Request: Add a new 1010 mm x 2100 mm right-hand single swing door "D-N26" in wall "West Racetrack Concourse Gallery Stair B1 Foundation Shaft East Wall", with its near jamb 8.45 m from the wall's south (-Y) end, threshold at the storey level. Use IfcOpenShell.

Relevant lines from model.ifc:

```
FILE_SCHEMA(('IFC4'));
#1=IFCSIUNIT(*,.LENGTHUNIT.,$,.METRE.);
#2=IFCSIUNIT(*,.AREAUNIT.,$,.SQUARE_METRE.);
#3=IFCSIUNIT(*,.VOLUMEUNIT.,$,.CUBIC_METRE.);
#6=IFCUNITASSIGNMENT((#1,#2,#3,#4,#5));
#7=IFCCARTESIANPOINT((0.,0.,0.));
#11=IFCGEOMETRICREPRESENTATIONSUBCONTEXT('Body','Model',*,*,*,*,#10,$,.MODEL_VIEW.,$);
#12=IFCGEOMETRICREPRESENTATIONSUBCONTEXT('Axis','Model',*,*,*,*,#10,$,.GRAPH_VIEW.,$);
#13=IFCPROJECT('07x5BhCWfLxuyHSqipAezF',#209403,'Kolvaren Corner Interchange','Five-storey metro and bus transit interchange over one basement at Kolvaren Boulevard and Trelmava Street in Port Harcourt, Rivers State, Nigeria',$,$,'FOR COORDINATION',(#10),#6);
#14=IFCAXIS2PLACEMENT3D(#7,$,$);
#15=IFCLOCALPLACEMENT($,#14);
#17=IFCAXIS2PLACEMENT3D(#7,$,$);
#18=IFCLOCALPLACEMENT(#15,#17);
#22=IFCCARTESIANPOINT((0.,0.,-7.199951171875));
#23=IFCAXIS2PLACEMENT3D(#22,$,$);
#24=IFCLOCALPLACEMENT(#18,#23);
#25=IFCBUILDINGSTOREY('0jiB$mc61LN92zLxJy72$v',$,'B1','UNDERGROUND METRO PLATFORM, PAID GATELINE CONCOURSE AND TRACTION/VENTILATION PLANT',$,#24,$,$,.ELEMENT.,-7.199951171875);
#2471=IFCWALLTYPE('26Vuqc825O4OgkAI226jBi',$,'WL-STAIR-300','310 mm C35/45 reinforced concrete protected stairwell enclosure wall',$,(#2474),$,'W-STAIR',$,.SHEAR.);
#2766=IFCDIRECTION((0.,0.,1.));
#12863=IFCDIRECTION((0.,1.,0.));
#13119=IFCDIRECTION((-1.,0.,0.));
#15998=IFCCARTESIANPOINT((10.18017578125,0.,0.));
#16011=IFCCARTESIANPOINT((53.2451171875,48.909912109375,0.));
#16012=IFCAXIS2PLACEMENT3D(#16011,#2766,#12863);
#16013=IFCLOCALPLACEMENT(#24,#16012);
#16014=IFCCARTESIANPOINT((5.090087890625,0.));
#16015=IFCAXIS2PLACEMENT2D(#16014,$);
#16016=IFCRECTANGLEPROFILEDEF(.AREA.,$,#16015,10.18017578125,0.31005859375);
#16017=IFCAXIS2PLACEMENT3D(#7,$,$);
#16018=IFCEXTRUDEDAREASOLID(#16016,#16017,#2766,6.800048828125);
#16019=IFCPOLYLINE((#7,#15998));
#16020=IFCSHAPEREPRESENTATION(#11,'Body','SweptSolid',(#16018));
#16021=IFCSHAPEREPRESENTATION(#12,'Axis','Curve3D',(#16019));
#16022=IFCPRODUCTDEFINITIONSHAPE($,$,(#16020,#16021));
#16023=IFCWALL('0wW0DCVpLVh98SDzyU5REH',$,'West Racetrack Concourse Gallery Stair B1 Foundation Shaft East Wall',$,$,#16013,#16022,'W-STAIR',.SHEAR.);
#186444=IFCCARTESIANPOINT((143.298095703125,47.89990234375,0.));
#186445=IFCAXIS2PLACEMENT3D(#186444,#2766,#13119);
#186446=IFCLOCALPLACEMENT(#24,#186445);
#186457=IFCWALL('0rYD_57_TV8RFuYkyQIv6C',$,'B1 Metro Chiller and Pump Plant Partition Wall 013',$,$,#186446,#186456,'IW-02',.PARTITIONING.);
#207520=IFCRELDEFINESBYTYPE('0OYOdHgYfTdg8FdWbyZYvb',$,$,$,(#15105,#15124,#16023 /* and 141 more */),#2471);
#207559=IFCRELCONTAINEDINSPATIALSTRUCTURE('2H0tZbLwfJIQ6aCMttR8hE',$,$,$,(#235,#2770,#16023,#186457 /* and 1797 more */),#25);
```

```python
import numpy as np
import ifcopenshell
import ifcopenshell.api.feature
import ifcopenshell.api.geometry
import ifcopenshell.api.root
import ifcopenshell.api.spatial
import ifcopenshell.geom
import ifcopenshell.util.element
import ifcopenshell.util.placement
import ifcopenshell.util.representation
import ifcopenshell.util.shape
import ifcopenshell.util.unit

model = ifcopenshell.open("model.ifc")
unit_scale = ifcopenshell.util.unit.calculate_unit_scale(model)
settings = ifcopenshell.geom.settings()


def volume(element):
    """Net volume in cubic metres, openings subtracted."""
    shape = ifcopenshell.geom.create_shape(settings, element)
    return ifcopenshell.util.shape.get_volume(shape.geometry)


wall = model.by_guid("0wW0DCVpLVh98SDzyU5REH")
storey = ifcopenshell.util.element.get_container(wall, ifc_class="IfcBuildingStorey")
context = ifcopenshell.util.representation.get_context(model, "Model", "Body", "MODEL_VIEW")
before = volume(wall)

width, height, from_end, sill = 1.01, 2.1, 8.45, 0.0  # metres

# The wall runs along its own X axis, and the end named is its -X end.
wall_shape = ifcopenshell.geom.create_shape(settings, wall)
x, y, z = ifcopenshell.util.shape.get_vertices(wall_shape.geometry).T
start = x.min() + from_end
face, thickness = float(y.min()), float(y.max() - y.min())
wall_matrix = ifcopenshell.util.placement.get_local_placement(wall.ObjectPlacement)
level = ifcopenshell.util.placement.get_local_placement(storey.ObjectPlacement)[2, 3]


def in_wall(x, y):
    """Placement at x, y metres in the wall's axes, at sill height."""
    matrix = wall_matrix.copy()
    matrix[:, 3] = wall_matrix @ np.array([x / unit_scale, y / unit_scale, 0.0, 1.0])
    matrix[2, 3] = level + sill / unit_scale
    return matrix


# Opening: a box that overshoots both wall faces by 50 mm.
opening = ifcopenshell.api.root.create_entity(model, ifc_class="IfcOpeningElement", predefined_type="OPENING")
box = ifcopenshell.api.geometry.add_wall_representation(
    model, context=context, length=width, height=height, thickness=thickness + 0.1
)
ifcopenshell.api.geometry.assign_representation(model, product=opening, representation=box)
ifcopenshell.api.geometry.edit_object_placement(model, product=opening, matrix=in_wall(start, face - 0.05), is_si=False)
ifcopenshell.api.feature.add_feature(model, feature=opening, element=wall)

door = ifcopenshell.api.root.create_entity(model, ifc_class="IfcDoor", name="D-N26", predefined_type="DOOR")
door.OverallWidth, door.OverallHeight = width / unit_scale, height / unit_scale
door.OperationType = "SINGLE_SWING_RIGHT"
body = ifcopenshell.api.geometry.add_door_representation(
    model,
    context=context,
    overall_width=door.OverallWidth,
    overall_height=door.OverallHeight,
    operation_type="SINGLE_SWING_RIGHT",
    lining_properties={"LiningDepth": thickness / unit_scale, "ThresholdDepth": thickness / unit_scale},
)
ifcopenshell.api.geometry.assign_representation(model, product=door, representation=body)
ifcopenshell.api.spatial.assign_container(model, products=[door], relating_structure=storey)
ifcopenshell.api.feature.add_filling(model, opening=opening, element=door)

# The lining spans the wall, so the door starts at the wall face.
ifcopenshell.api.geometry.edit_object_placement(model, product=door, matrix=in_wall(start, face), is_si=False)

after = volume(wall)

print(f"wall volume {before:.3f} -> {after:.3f} m3")

model.write("model_edited.ifc")
```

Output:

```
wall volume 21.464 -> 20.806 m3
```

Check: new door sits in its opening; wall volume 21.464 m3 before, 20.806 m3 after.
